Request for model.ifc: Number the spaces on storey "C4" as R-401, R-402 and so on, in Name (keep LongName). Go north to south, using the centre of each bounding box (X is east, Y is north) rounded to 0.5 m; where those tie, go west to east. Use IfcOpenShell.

First a look at what the model holds.

```python
import ifcopenshell
import ifcopenshell.util.element
import ifcopenshell.util.placement

model = ifcopenshell.open("model.ifc")
print(model.schema)
storey = next(s for s in model.by_type("IfcBuildingStorey") if s.Name == "C4")
spaces = [e for e in ifcopenshell.util.element.get_decomposition(storey) if e.is_a("IfcSpace")]
for e in sorted(spaces, key=lambda e: e.id()):
    origin = ifcopenshell.util.placement.get_local_placement(e.ObjectPlacement)[:3, 3]
    print(e.id(), e.Name, e.LongName, origin.round(2) + 0.0, sep=" | ")
```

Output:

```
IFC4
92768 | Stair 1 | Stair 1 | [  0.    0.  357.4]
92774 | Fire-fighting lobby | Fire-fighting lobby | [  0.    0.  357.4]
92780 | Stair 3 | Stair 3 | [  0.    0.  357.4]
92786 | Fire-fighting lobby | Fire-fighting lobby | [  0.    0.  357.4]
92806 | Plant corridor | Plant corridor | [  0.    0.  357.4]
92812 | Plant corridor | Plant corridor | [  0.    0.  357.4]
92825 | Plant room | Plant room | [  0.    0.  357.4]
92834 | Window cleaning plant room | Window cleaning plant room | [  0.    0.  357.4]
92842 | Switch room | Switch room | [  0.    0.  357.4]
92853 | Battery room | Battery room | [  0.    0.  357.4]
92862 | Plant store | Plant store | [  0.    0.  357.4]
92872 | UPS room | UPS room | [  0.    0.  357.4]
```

```python
import ifcopenshell
import ifcopenshell.geom
import ifcopenshell.util.element
import ifcopenshell.util.shape

model = ifcopenshell.open("model.ifc")
settings = ifcopenshell.geom.settings()
settings.set("use-world-coords", True)


def centre(element):
    shape = ifcopenshell.geom.create_shape(settings, element)
    return ifcopenshell.util.shape.get_bbox_centroid(shape.geometry)


storey = next(s for s in model.by_type("IfcBuildingStorey") if s.Name == "C4")
spaces = [e for e in ifcopenshell.util.element.get_decomposition(storey) if e.is_a("IfcSpace")]

# Insertion points can sit at a corner or the storey origin, so sort by the geometry (in metres).
centres = {e: centre(e) for e in spaces}
spaces.sort(key=lambda e: (-round(centres[e][1] / 0.5), centres[e][0]))

for i, e in enumerate(spaces, start=1):
    number = f"R-4{i:02d}"
    e.Name = number
    print(e.id(), number)

model.write("model_v2.ifc")
```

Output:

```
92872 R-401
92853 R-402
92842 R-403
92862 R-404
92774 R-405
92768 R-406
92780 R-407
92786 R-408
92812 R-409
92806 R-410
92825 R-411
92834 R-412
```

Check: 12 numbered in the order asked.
